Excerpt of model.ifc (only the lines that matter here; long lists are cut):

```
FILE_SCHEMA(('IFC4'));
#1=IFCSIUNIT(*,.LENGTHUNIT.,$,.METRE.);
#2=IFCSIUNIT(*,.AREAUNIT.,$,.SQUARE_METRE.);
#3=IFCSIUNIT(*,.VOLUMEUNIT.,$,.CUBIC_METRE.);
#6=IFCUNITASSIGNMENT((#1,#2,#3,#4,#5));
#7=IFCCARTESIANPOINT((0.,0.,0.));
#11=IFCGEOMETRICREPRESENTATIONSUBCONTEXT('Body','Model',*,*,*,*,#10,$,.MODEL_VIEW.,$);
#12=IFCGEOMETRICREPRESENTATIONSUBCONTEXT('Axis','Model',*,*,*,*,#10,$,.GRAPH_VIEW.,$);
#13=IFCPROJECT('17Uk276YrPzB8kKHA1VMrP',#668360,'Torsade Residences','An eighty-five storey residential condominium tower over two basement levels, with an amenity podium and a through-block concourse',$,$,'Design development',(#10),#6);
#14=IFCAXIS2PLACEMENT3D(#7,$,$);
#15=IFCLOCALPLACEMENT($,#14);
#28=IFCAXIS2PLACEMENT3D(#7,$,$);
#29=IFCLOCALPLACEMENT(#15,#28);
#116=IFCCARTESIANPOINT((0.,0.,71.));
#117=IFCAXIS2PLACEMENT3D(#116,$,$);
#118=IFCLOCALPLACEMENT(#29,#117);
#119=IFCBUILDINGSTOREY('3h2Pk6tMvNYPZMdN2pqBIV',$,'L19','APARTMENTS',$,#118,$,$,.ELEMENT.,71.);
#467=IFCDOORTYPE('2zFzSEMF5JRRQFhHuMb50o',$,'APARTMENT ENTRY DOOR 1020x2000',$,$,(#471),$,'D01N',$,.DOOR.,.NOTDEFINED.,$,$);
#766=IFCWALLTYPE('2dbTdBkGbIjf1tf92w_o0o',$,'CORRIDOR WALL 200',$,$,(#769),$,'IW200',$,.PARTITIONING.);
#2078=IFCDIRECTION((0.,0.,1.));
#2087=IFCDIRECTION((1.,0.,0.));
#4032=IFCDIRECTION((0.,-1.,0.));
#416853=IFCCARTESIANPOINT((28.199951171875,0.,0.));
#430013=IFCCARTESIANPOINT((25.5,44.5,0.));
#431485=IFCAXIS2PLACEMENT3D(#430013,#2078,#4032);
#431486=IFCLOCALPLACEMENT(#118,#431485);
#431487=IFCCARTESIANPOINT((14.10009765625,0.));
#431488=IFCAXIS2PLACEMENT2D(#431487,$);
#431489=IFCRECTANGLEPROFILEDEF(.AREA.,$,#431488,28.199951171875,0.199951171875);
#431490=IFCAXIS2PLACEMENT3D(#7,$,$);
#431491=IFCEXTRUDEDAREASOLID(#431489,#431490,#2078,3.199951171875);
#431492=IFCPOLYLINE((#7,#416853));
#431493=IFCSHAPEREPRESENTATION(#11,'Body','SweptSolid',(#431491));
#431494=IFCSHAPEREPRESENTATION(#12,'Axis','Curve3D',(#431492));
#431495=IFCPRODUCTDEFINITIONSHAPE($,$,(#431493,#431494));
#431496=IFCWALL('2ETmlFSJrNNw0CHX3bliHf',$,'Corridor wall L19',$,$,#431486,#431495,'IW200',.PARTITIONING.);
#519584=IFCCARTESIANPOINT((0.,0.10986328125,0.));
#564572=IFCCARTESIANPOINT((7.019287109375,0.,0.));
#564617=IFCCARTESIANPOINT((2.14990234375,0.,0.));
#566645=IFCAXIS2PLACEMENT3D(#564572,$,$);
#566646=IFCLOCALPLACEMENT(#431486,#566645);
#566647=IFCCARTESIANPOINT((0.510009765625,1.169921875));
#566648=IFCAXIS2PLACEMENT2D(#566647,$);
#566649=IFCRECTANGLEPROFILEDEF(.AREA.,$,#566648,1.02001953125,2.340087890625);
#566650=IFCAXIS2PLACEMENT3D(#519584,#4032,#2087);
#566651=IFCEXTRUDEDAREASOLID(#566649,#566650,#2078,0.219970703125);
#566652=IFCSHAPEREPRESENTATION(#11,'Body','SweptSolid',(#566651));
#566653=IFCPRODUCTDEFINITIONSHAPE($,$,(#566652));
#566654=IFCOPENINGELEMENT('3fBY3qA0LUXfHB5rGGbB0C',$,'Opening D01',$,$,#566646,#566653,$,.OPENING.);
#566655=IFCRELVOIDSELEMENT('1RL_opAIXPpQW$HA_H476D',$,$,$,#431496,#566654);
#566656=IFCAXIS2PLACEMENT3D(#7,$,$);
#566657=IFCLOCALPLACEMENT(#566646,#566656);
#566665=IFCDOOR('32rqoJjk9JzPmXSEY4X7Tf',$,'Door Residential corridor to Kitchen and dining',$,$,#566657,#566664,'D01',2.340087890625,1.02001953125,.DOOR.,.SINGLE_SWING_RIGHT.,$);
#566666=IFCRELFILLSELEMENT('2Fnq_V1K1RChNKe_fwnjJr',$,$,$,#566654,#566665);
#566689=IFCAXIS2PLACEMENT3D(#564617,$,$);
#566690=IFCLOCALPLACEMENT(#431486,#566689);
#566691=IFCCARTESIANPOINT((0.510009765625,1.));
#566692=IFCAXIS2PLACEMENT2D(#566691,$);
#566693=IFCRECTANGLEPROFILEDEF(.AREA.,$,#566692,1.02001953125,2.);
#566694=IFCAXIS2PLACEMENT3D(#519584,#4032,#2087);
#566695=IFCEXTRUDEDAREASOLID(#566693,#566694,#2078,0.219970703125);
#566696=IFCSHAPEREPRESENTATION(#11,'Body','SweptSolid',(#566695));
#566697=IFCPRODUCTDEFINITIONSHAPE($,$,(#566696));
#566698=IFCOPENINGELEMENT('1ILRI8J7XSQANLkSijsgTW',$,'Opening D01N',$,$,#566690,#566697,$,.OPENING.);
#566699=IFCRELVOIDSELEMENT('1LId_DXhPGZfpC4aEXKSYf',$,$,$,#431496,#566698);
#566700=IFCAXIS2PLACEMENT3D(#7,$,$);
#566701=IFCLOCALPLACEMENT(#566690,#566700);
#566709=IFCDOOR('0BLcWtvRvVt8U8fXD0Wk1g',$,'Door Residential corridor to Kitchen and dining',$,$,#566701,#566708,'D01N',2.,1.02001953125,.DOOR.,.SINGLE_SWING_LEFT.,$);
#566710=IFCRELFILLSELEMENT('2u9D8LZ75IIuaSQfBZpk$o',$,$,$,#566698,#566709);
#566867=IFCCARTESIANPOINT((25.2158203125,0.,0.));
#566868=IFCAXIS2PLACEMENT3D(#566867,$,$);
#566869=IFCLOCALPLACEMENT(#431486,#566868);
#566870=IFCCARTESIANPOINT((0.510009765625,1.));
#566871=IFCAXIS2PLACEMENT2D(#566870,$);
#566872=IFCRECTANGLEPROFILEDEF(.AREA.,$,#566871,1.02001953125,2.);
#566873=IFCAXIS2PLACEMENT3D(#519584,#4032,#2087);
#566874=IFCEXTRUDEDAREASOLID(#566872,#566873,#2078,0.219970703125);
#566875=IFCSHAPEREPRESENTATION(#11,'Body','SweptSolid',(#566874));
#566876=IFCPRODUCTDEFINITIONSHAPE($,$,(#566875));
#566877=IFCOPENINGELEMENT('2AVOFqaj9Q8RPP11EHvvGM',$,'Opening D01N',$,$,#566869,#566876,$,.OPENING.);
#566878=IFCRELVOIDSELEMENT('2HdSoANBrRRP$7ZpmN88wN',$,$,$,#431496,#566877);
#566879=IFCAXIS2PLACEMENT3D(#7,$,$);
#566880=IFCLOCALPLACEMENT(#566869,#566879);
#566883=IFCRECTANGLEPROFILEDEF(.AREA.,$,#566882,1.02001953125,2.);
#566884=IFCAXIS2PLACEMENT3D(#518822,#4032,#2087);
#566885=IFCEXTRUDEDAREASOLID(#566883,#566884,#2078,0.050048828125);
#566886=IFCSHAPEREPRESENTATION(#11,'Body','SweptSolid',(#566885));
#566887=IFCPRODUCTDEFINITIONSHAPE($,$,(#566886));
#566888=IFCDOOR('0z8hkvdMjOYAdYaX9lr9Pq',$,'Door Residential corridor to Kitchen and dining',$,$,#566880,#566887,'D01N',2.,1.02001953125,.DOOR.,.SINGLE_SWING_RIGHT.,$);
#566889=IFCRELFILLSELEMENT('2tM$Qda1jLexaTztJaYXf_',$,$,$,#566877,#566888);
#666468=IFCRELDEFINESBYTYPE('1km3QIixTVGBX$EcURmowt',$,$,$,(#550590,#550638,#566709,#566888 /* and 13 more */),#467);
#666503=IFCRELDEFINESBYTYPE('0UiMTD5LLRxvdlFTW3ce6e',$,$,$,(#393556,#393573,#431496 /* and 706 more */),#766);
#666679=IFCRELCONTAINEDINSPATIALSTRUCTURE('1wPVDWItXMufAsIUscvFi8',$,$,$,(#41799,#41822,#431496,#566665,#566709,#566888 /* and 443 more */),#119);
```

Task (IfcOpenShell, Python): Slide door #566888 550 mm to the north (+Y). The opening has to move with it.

```python
import ifcopenshell
import ifcopenshell.api.geometry
import ifcopenshell.util.placement

model = ifcopenshell.open("model.ifc")

door = model.by_guid("0z8hkvdMjOYAdYaX9lr9Pq")
opening = door.FillsVoids[0].RelatingOpeningElement
wall = opening.VoidsElements[0].RelatingBuildingElement

wall_matrix = ifcopenshell.util.placement.get_local_placement(wall.ObjectPlacement)
shift = wall_matrix[:3, 0] * -0.55
before = ifcopenshell.util.placement.get_local_placement(door.ObjectPlacement)[:3, 3].copy()

# The door is placed relative to its opening, so it follows when the opening moves.
matrix = ifcopenshell.util.placement.get_local_placement(opening.ObjectPlacement)
matrix[:3, 3] += shift
ifcopenshell.api.geometry.edit_object_placement(
    model, product=opening, matrix=matrix, is_si=False, should_transform_children=True
)

after = ifcopenshell.util.placement.get_local_placement(door.ObjectPlacement)[:3, 3]
print("door moved by", (after - before).round(3) + 0.0)

model.write("model_rev.ifc")
```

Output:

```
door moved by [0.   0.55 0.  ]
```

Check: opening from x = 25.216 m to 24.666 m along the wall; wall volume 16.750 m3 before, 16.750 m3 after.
